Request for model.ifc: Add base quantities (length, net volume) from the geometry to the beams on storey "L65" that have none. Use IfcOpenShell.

First a look at what the model holds.

```python
import ifcopenshell
import ifcopenshell.util.element
import ifcopenshell.util.unit

model = ifcopenshell.open("model.ifc")
print(model.schema)
for unit_type in ("LENGTHUNIT", "AREAUNIT", "VOLUMEUNIT"):
    print(unit_type, ifcopenshell.util.unit.calculate_unit_scale(model, unit_type))
storey = next(s for s in model.by_type("IfcBuildingStorey") if s.Name == "L65")
beams = [e for e in ifcopenshell.util.element.get_decomposition(storey) if e.is_a("IfcBeam")]
for e in sorted(beams, key=lambda e: e.id()):
    print(e.id(), e.is_a(), e.Name, list(ifcopenshell.util.element.get_psets(e, qtos_only=True)), sep=" | ")
```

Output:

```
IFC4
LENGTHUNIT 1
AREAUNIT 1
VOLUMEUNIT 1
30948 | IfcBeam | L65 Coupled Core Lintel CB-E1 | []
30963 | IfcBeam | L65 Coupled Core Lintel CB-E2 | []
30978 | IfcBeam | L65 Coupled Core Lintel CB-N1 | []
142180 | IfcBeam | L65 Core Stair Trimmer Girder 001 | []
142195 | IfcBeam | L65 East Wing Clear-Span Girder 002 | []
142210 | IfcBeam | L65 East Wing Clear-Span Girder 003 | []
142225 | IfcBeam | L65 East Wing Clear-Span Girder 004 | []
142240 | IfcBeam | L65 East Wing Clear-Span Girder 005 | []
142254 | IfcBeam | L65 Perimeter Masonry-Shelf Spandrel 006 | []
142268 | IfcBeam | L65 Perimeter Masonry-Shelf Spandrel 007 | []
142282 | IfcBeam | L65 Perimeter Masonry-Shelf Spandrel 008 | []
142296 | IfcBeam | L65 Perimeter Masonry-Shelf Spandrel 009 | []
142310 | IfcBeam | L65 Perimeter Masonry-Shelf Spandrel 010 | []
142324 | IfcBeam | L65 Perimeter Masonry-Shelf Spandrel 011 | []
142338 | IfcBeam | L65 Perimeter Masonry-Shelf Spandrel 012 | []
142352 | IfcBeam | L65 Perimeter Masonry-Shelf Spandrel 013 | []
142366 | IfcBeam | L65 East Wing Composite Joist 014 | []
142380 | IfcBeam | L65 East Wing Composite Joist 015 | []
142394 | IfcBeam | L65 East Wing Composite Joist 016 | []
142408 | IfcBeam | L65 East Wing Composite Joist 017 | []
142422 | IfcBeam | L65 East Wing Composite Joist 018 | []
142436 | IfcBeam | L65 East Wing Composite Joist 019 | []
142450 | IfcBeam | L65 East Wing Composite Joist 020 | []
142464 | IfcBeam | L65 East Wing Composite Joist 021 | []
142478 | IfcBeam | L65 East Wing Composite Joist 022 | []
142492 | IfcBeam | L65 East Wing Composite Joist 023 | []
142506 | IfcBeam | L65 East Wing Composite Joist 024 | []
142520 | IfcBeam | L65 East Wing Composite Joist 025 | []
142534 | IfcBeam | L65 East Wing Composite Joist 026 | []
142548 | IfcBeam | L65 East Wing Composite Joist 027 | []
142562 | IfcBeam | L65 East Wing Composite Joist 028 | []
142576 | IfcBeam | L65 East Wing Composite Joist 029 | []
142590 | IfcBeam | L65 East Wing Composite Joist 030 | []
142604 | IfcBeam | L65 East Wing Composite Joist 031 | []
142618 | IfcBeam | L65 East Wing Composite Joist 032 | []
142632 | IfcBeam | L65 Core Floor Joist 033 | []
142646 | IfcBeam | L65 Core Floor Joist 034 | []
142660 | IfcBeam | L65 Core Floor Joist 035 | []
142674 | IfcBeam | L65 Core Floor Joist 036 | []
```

```python
import ifcopenshell
import ifcopenshell.api.pset
import ifcopenshell.geom
import ifcopenshell.util.element
import ifcopenshell.util.shape
import ifcopenshell.util.unit

model = ifcopenshell.open("model.ifc")
unit_scale = ifcopenshell.util.unit.calculate_unit_scale(model)
volume_scale = ifcopenshell.util.unit.calculate_unit_scale(model, "VOLUMEUNIT")
settings = ifcopenshell.geom.settings()

storey = next(s for s in model.by_type("IfcBuildingStorey") if s.Name == "L65")
beams = [e for e in ifcopenshell.util.element.get_decomposition(storey) if e.is_a("IfcBeam")]

for e in sorted(beams, key=lambda e: e.id()):
    if ifcopenshell.util.element.get_psets(e, qtos_only=True, should_inherit=False):
        continue
    # Geometry comes back in metres, in the element's own axes.
    shape = ifcopenshell.geom.create_shape(settings, e)
    values = {
        "Length": ifcopenshell.util.shape.get_max_xyz(shape.geometry) / unit_scale,
        "NetVolume": ifcopenshell.util.shape.get_volume(shape.geometry) / volume_scale,
    }
    qto = ifcopenshell.api.pset.add_qto(model, product=e, name="Qto_BeamBaseQuantities")
    ifcopenshell.api.pset.edit_qto(model, qto=qto, properties=values)
    print(e.id(), {k: round(v, 3) for k, v in values.items()})

model.write("model_rev.ifc")
```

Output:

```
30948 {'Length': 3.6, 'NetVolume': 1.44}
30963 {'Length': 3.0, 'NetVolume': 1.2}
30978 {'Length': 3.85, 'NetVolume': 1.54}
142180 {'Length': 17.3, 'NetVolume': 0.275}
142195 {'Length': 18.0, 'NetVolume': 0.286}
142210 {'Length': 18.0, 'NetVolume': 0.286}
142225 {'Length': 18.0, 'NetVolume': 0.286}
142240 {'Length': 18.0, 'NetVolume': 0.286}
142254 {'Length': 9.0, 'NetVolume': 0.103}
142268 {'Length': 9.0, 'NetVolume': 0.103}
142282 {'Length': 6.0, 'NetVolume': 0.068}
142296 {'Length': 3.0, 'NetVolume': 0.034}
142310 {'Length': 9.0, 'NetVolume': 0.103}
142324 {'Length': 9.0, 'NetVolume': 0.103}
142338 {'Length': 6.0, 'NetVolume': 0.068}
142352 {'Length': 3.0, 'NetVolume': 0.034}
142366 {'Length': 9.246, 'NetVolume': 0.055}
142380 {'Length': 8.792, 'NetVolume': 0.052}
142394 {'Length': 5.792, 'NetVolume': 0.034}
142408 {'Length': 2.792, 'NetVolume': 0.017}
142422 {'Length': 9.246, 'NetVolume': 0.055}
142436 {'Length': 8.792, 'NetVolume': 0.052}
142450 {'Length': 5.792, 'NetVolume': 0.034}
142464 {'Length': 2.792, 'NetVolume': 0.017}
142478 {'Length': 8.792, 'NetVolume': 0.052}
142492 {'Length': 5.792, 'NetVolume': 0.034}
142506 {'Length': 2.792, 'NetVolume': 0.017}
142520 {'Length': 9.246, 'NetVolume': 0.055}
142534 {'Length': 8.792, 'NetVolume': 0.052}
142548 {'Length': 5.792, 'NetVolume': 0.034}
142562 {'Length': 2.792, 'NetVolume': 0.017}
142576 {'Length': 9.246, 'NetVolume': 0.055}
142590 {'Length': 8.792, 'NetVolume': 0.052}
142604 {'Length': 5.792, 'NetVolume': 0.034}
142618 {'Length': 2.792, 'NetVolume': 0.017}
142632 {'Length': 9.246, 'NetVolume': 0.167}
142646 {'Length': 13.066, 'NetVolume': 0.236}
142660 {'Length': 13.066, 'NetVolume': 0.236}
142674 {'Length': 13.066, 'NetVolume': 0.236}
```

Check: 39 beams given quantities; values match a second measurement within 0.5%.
